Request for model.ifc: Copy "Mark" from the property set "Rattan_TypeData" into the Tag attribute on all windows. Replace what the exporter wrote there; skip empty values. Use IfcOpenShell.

First a look at what the model holds.

```python
import ifcopenshell
import ifcopenshell.util.element

model = ifcopenshell.open("model.ifc")
print(model.schema)
windows = model.by_type("IfcWindow")
print(len(windows), "windows")
for e in windows[:8]:
    source = ifcopenshell.util.element.get_pset(e, "Rattan_TypeData", "Mark")
    target = e.Tag
    print(e.id(), repr(source), repr(target), sep=" | ")
```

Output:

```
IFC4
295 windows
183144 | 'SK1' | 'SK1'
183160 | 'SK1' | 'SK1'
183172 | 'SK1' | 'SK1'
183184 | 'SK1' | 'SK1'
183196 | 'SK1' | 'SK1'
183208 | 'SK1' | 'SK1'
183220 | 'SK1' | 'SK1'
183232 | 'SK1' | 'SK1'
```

```python
import ifcopenshell
import ifcopenshell.util.element

model = ifcopenshell.open("model.ifc")

count = 0
for e in model.by_type("IfcWindow"):
    value = ifcopenshell.util.element.get_pset(e, "Rattan_TypeData", "Mark")
    current = e.Tag
    if not value or not value.strip() or current == value:
        continue
    e.Tag = value
    count += 1

print(count, "windows updated")

model.write("model_edited.ifc")
```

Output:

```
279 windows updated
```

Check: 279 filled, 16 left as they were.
